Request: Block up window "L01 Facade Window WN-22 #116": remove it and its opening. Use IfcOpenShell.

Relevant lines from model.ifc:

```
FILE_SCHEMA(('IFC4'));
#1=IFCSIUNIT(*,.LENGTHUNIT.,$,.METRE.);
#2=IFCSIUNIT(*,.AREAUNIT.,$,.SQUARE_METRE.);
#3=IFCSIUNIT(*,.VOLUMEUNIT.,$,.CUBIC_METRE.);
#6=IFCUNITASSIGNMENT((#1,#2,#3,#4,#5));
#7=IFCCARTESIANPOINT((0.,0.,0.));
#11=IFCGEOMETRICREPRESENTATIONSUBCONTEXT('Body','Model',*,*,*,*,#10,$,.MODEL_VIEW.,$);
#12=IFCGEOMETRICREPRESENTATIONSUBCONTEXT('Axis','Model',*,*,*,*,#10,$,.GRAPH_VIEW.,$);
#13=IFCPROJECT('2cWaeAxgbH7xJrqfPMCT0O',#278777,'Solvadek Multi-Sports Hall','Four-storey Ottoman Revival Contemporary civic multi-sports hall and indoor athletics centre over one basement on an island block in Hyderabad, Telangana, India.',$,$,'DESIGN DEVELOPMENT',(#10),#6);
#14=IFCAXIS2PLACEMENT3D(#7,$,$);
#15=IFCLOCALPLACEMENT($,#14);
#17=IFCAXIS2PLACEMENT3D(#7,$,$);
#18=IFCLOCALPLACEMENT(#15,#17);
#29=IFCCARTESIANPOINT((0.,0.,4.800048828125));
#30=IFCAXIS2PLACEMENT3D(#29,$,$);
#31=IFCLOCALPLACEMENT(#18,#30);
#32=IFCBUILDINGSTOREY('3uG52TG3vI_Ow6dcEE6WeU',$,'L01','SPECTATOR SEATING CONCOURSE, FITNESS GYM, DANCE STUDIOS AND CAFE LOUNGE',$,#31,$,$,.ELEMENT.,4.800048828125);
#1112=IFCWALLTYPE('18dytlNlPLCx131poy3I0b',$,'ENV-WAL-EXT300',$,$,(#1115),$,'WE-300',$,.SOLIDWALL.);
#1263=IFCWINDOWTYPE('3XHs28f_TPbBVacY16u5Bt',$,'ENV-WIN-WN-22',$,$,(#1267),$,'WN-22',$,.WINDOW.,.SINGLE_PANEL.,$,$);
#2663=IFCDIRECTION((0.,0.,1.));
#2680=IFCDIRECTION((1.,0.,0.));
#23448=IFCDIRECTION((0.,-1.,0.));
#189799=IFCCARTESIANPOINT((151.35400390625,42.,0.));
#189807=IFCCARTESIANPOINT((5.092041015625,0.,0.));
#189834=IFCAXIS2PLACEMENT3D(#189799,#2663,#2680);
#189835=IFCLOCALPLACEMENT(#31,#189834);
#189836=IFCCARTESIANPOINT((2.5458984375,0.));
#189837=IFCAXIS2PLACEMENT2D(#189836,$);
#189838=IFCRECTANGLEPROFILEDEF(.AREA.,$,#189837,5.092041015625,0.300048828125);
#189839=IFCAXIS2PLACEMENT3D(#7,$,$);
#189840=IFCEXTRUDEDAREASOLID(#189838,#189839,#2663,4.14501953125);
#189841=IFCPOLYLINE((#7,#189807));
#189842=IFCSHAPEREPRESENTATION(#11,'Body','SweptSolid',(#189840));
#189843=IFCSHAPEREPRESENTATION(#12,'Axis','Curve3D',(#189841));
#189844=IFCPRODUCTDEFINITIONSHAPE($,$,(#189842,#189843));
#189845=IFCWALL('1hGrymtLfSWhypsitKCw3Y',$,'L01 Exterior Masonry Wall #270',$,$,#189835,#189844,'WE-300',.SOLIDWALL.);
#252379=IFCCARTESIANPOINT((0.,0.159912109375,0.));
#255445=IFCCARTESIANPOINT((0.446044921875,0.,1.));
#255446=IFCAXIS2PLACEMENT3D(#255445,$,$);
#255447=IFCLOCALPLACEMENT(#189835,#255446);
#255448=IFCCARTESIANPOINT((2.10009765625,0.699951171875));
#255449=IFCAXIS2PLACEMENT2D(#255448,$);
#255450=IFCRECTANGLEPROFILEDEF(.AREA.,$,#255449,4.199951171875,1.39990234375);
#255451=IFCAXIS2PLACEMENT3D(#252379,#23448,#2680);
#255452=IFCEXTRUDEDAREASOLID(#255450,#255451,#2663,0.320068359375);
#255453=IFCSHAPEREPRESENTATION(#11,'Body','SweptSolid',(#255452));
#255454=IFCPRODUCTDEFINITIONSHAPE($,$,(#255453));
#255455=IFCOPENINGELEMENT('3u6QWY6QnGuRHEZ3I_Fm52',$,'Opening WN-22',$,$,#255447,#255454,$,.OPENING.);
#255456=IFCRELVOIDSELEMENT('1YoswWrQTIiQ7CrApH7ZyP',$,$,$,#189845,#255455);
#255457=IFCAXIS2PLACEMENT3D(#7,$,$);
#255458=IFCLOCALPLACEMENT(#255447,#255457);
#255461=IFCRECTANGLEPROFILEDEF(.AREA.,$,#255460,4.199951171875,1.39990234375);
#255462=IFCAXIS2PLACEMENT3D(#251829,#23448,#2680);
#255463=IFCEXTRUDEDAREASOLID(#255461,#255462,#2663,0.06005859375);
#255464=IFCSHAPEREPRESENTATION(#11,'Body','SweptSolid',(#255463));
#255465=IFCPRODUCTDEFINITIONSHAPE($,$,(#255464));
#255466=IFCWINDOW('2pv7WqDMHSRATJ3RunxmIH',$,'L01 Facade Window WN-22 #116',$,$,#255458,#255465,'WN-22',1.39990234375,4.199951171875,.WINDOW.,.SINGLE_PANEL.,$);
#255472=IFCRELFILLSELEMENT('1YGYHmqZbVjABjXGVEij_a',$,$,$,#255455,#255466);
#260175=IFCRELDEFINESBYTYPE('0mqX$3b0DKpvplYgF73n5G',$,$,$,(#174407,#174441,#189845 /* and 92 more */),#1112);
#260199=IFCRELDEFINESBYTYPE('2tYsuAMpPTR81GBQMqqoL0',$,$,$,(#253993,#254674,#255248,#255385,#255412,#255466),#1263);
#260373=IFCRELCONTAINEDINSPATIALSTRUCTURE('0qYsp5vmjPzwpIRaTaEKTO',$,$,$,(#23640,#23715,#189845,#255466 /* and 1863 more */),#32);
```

```python
import ifcopenshell
import ifcopenshell.api.feature
import ifcopenshell.api.root
import ifcopenshell.geom
import ifcopenshell.util.shape

model = ifcopenshell.open("model.ifc")
settings = ifcopenshell.geom.settings()


def volume(element):
    """Net volume in cubic metres, openings subtracted."""
    shape = ifcopenshell.geom.create_shape(settings, element)
    return ifcopenshell.util.shape.get_volume(shape.geometry)


window = model.by_guid("2pv7WqDMHSRATJ3RunxmIH")
opening = window.FillsVoids[0].RelatingOpeningElement
wall = opening.VoidsElements[0].RelatingBuildingElement
before = volume(wall)

ifcopenshell.api.root.remove_product(model, product=window)
ifcopenshell.api.feature.remove_feature(model, feature=opening)

after = volume(wall)

print(f"wall volume {before:.3f} -> {after:.3f} m3")

model.write("model_v2.ifc")
```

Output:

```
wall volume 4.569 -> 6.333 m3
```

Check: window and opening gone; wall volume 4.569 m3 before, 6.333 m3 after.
